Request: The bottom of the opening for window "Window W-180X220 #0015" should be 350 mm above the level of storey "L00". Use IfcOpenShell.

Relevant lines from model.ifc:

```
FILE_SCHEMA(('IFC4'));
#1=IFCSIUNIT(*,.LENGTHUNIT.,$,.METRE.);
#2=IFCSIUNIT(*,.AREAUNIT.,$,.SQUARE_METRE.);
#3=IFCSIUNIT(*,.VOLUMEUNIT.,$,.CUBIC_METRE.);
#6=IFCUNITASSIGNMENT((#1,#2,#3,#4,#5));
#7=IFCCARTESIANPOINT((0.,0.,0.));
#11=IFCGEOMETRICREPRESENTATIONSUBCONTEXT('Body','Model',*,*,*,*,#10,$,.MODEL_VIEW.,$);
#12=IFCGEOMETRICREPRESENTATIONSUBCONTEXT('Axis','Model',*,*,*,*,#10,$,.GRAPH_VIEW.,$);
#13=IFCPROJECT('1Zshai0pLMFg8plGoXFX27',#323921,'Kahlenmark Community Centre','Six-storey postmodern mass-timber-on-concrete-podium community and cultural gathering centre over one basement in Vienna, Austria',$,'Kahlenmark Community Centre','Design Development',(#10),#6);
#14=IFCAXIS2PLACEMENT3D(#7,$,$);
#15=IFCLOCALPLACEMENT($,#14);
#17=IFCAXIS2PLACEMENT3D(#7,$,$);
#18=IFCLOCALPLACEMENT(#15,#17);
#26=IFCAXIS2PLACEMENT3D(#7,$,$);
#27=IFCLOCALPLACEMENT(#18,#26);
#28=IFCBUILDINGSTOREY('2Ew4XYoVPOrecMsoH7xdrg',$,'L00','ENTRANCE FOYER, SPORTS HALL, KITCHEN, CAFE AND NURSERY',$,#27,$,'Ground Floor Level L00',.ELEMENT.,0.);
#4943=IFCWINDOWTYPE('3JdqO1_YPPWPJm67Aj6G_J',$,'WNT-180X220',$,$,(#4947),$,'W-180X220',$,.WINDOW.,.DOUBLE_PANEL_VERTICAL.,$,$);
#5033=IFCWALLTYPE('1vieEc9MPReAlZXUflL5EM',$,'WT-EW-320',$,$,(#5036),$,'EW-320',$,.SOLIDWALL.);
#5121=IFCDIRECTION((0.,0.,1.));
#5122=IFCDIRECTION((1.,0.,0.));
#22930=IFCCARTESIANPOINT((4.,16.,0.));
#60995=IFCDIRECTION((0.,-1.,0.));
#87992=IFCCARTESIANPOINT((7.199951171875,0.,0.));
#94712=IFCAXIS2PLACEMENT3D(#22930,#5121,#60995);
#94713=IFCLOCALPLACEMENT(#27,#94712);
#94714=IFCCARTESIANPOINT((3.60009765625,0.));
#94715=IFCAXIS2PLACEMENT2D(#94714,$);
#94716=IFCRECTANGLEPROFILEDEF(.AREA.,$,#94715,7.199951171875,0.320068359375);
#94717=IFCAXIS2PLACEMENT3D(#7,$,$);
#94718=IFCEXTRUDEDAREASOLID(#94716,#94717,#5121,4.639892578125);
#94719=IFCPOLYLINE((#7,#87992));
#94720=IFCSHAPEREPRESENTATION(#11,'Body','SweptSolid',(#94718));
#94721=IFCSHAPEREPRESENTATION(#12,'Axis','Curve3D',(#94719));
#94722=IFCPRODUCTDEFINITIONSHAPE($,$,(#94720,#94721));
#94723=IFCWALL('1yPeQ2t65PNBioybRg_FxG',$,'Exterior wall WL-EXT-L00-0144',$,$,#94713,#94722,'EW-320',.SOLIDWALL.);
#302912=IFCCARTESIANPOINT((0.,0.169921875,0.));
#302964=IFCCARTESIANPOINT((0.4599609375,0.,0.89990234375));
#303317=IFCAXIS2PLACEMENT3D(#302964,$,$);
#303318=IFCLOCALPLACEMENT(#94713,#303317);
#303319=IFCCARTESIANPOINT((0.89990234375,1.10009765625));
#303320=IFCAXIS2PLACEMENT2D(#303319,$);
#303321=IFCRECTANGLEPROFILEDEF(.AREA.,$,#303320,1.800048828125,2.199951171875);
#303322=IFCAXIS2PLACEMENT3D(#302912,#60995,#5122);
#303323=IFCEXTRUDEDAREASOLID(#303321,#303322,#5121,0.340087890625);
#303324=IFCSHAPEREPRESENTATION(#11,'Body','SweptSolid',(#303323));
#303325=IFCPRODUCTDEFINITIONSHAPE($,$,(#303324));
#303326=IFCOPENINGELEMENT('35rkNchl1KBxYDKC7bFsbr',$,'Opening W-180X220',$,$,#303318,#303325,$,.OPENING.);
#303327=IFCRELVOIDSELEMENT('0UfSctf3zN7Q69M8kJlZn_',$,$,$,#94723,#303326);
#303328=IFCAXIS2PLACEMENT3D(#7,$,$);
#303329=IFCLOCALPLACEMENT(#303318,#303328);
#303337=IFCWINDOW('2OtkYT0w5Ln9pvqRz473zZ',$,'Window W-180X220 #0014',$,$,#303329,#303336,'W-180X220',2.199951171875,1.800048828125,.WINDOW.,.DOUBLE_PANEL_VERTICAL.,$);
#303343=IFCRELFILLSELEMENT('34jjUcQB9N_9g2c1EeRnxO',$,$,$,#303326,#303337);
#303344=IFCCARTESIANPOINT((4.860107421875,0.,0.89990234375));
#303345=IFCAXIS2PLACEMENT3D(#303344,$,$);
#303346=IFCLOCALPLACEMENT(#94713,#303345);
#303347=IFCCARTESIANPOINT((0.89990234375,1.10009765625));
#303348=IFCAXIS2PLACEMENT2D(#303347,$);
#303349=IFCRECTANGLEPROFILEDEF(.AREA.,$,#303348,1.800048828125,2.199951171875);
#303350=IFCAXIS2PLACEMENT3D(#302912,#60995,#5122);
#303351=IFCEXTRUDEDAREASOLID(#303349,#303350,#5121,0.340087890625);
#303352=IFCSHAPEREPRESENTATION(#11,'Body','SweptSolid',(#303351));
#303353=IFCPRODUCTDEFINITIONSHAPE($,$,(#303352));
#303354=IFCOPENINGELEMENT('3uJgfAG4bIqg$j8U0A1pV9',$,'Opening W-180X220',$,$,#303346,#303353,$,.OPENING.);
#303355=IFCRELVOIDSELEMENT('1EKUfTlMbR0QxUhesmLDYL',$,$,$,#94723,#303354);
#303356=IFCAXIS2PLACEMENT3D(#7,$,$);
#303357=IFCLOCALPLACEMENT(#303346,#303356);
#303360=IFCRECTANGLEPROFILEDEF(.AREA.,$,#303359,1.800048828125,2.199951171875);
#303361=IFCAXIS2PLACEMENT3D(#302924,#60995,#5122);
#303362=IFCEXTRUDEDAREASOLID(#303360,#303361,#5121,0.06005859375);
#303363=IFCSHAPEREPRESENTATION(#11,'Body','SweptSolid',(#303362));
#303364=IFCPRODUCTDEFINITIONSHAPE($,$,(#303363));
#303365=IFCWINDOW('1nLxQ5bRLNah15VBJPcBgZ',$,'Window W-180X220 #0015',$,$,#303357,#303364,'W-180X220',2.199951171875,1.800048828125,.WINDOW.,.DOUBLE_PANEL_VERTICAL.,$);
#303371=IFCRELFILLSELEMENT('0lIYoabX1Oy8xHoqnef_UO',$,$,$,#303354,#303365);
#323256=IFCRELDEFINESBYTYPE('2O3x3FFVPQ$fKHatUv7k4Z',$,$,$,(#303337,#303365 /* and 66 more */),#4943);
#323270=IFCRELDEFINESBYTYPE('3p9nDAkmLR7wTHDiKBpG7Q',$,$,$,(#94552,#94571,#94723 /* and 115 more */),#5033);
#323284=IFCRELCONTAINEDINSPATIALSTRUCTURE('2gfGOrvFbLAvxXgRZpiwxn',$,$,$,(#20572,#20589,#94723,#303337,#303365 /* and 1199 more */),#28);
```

```python
import numpy as np
import ifcopenshell
import ifcopenshell.api.geometry
import ifcopenshell.geom
import ifcopenshell.util.element
import ifcopenshell.util.placement
import ifcopenshell.util.shape
import ifcopenshell.util.unit

model = ifcopenshell.open("model.ifc")
unit_scale = ifcopenshell.util.unit.calculate_unit_scale(model)

window = model.by_id(303365)
opening = window.FillsVoids[0].RelatingOpeningElement
storey = ifcopenshell.util.element.get_container(window, ifc_class="IfcBuildingStorey")
level = ifcopenshell.util.placement.get_local_placement(storey.ObjectPlacement)[2, 3]

# The opening's origin need not be at the sill, so measure its lowest point.
shape = ifcopenshell.geom.create_shape(ifcopenshell.geom.settings(), opening)
bottom = ifcopenshell.util.shape.get_shape_bottom_elevation(shape, shape.geometry) / unit_scale
dz = level + 0.35 / unit_scale - bottom

shift = np.array([0.0, 0.0, dz])
# The window is placed relative to its opening, so it follows when the opening moves.
matrix = ifcopenshell.util.placement.get_local_placement(opening.ObjectPlacement)
matrix[:3, 3] += shift
ifcopenshell.api.geometry.edit_object_placement(
    model, product=opening, matrix=matrix, is_si=False, should_transform_children=True
)

print(f"moved by {dz * unit_scale:+.3f} m")

model.write("model_edited.ifc")
```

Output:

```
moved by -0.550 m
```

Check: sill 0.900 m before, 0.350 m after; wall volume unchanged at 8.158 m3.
